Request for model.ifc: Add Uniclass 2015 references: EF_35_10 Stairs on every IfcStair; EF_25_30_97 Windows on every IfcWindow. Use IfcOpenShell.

First a look at what the model holds.

```python
import ifcopenshell

model = ifcopenshell.open("model.ifc")
print(model.schema)
print("classifications:", [c.Name for c in model.by_type("IfcClassification")])
for ifc_class in ("IfcDoor", "IfcRoof", "IfcStair", "IfcWall", "IfcWindow"):
    print(ifc_class, len(model.by_type(ifc_class)))
```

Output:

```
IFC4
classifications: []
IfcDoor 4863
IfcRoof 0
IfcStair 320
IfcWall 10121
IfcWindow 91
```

```python
import ifcopenshell
import ifcopenshell.api.classification

model = ifcopenshell.open("model.ifc")

system = ifcopenshell.api.classification.add_classification(model, classification="Uniclass 2015")

codes = {
    "IfcStair": ("EF_35_10", "Stairs"),
    "IfcWindow": ("EF_25_30_97", "Windows"),
}
for ifc_class, (code, name) in codes.items():
    products = model.by_type(ifc_class)
    ifcopenshell.api.classification.add_reference(
        model, products=products, classification=system, identification=code, name=name
    )
    print(code, len(products))

model.write("model_v2.ifc")
```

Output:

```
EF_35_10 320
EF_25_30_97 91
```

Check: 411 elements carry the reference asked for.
